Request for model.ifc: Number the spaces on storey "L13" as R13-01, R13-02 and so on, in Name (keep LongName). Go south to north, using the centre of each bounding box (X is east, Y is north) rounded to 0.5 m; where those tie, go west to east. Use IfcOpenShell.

First a look at what the model holds.

```python
import ifcopenshell
import ifcopenshell.util.element
import ifcopenshell.util.placement

model = ifcopenshell.open("model.ifc")
print(model.schema)
storey = next(s for s in model.by_type("IfcBuildingStorey") if s.Name == "L13")
spaces = [e for e in ifcopenshell.util.element.get_decomposition(storey) if e.is_a("IfcSpace")]
for e in sorted(spaces, key=lambda e: e.id()):
    origin = ifcopenshell.util.placement.get_local_placement(e.ObjectPlacement)[:3, 3]
    print(e.id(), e.Name, e.LongName, origin.round(2) + 0.0, sep=" | ")
```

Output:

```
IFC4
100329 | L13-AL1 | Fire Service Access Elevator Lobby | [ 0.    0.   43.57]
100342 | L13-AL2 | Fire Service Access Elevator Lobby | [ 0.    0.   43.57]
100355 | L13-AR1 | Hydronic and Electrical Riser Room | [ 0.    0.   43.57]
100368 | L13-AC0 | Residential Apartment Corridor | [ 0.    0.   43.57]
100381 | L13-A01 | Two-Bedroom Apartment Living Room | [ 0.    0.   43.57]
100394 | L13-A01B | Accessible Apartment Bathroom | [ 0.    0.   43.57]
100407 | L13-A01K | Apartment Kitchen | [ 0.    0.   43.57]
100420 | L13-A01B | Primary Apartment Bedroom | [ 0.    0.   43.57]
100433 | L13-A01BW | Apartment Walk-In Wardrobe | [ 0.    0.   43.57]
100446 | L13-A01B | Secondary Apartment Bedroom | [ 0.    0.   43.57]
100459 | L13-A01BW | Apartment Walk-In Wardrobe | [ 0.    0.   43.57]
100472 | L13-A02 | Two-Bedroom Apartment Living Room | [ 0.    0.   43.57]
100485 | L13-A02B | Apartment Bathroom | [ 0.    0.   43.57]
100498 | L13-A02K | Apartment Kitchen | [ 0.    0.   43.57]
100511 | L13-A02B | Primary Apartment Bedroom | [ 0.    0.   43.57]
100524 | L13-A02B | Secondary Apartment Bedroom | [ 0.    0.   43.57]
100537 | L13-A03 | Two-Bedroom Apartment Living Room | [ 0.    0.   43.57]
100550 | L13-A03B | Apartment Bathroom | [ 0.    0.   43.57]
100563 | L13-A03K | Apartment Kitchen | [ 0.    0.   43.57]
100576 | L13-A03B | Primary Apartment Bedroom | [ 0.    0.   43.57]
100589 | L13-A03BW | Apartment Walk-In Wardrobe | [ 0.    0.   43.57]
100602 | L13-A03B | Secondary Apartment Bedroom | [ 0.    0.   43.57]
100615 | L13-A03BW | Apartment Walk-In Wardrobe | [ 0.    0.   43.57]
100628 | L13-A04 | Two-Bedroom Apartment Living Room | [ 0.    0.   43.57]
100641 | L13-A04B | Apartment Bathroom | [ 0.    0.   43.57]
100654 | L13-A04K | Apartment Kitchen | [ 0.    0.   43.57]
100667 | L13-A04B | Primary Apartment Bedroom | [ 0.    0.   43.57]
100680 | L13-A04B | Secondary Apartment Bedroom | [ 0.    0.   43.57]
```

```python
import ifcopenshell
import ifcopenshell.geom
import ifcopenshell.util.element
import ifcopenshell.util.shape

model = ifcopenshell.open("model.ifc")
settings = ifcopenshell.geom.settings()
settings.set("use-world-coords", True)


def centre(element):
    shape = ifcopenshell.geom.create_shape(settings, element)
    return ifcopenshell.util.shape.get_bbox_centroid(shape.geometry)


storey = next(s for s in model.by_type("IfcBuildingStorey") if s.Name == "L13")
spaces = [e for e in ifcopenshell.util.element.get_decomposition(storey) if e.is_a("IfcSpace")]

# Insertion points can sit at a corner or the storey origin, so sort by the geometry (in metres).
centres = {e: centre(e) for e in spaces}
spaces.sort(key=lambda e: (round(centres[e][1] / 0.5), centres[e][0]))

for i, e in enumerate(spaces, start=1):
    number = f"R13-{i:02d}"
    e.Name = number
    print(e.id(), number)

model.write("model-out.ifc")
```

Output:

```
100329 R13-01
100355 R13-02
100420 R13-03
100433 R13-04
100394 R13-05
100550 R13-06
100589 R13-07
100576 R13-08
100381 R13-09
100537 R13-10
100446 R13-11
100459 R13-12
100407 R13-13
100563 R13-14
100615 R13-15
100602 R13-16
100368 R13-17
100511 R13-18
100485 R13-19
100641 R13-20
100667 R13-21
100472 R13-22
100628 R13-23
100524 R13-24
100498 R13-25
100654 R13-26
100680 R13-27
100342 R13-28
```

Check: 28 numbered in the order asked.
